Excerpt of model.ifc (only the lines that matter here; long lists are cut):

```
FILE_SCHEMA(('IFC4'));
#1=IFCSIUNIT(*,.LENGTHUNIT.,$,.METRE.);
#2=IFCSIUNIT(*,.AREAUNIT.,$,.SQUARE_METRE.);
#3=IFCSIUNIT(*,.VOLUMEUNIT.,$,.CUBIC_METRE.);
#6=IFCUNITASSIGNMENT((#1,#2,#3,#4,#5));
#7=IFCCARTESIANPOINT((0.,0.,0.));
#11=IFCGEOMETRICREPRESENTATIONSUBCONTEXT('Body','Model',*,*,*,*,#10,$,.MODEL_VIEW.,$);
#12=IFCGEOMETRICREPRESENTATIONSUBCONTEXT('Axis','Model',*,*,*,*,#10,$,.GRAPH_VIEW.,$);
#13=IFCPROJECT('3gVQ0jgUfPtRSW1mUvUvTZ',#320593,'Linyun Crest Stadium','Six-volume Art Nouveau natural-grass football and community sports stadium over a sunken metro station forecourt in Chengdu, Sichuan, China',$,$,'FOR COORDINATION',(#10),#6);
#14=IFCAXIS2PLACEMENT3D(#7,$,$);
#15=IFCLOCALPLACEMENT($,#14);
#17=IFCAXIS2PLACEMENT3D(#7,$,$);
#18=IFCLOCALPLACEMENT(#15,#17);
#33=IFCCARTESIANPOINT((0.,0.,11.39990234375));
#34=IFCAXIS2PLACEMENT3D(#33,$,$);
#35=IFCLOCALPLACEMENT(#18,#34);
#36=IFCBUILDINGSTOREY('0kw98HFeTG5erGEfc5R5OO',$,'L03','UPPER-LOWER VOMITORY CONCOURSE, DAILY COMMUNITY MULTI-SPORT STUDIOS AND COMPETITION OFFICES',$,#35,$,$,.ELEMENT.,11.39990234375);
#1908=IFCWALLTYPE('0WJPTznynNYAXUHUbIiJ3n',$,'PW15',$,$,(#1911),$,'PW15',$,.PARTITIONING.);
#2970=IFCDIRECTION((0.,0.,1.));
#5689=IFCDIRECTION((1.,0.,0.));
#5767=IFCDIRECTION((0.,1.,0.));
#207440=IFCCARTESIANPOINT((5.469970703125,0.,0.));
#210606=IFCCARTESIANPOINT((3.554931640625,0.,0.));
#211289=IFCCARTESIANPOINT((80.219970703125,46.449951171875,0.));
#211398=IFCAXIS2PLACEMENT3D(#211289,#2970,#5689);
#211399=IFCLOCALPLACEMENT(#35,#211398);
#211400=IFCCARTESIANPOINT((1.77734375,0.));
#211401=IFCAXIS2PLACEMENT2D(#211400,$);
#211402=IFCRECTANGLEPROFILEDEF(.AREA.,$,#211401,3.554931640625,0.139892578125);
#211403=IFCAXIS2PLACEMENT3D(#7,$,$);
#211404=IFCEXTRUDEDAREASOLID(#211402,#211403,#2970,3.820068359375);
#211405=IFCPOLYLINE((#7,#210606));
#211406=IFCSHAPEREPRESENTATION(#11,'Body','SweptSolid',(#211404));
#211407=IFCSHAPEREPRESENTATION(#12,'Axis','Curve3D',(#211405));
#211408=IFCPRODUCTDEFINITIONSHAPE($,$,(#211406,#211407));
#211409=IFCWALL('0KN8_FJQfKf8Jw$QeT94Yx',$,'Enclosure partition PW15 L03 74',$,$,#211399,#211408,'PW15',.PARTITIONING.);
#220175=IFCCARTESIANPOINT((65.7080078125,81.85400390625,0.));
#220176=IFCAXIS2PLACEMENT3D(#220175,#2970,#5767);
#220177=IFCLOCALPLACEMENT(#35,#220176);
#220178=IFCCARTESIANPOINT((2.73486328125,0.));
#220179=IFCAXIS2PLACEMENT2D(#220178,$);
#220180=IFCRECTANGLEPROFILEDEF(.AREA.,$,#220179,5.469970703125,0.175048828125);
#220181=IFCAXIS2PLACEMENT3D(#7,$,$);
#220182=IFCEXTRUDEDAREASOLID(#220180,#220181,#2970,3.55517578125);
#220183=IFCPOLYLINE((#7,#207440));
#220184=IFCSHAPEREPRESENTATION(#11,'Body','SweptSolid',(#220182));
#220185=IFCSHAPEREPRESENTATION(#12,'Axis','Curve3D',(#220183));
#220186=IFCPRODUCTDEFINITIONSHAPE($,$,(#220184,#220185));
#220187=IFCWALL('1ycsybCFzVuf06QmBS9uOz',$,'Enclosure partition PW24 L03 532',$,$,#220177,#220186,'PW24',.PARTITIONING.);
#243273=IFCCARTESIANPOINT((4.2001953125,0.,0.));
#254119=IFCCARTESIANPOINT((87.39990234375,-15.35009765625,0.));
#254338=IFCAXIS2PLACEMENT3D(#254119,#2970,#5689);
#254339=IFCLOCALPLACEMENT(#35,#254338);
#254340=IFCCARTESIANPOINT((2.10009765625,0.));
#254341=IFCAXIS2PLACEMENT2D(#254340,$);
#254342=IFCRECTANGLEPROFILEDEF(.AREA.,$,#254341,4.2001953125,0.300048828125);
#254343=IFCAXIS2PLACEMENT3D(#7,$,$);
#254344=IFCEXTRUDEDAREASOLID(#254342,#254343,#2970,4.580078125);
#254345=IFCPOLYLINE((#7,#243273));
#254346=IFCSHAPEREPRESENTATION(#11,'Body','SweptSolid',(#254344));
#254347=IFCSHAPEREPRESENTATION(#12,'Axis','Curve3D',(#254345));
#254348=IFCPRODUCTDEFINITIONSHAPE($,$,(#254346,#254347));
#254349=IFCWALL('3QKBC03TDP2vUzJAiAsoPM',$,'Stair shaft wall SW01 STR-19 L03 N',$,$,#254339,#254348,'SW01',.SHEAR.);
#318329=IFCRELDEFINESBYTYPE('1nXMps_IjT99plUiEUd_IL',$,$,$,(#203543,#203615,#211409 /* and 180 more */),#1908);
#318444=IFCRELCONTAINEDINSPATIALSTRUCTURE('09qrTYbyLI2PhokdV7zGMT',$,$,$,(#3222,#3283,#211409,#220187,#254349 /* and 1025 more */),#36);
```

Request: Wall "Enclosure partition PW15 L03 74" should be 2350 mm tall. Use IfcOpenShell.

```python
import ifcopenshell
import ifcopenshell.geom
import ifcopenshell.util.representation
import ifcopenshell.util.shape
import ifcopenshell.util.unit

model = ifcopenshell.open("model.ifc")
unit_scale = ifcopenshell.util.unit.calculate_unit_scale(model)
settings = ifcopenshell.geom.settings()


def volume(element):
    """Net volume in cubic metres, openings subtracted."""
    shape = ifcopenshell.geom.create_shape(settings, element)
    return ifcopenshell.util.shape.get_volume(shape.geometry)


wall = model.by_guid("0KN8_FJQfKf8Jw$QeT94Yx")
before = volume(wall)

body = ifcopenshell.util.representation.get_representation(wall, "Model", "Body")
solid = body.Items[0]
old_height = solid.Depth
solid.Depth = 2.35 / unit_scale
after = volume(wall)

print(f"height {old_height:g} -> {solid.Depth:g}, volume {before:.3f} -> {after:.3f} m3")

model.write("model_updated.ifc")
```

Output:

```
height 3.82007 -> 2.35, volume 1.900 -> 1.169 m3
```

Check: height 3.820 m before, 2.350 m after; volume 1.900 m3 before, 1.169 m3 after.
